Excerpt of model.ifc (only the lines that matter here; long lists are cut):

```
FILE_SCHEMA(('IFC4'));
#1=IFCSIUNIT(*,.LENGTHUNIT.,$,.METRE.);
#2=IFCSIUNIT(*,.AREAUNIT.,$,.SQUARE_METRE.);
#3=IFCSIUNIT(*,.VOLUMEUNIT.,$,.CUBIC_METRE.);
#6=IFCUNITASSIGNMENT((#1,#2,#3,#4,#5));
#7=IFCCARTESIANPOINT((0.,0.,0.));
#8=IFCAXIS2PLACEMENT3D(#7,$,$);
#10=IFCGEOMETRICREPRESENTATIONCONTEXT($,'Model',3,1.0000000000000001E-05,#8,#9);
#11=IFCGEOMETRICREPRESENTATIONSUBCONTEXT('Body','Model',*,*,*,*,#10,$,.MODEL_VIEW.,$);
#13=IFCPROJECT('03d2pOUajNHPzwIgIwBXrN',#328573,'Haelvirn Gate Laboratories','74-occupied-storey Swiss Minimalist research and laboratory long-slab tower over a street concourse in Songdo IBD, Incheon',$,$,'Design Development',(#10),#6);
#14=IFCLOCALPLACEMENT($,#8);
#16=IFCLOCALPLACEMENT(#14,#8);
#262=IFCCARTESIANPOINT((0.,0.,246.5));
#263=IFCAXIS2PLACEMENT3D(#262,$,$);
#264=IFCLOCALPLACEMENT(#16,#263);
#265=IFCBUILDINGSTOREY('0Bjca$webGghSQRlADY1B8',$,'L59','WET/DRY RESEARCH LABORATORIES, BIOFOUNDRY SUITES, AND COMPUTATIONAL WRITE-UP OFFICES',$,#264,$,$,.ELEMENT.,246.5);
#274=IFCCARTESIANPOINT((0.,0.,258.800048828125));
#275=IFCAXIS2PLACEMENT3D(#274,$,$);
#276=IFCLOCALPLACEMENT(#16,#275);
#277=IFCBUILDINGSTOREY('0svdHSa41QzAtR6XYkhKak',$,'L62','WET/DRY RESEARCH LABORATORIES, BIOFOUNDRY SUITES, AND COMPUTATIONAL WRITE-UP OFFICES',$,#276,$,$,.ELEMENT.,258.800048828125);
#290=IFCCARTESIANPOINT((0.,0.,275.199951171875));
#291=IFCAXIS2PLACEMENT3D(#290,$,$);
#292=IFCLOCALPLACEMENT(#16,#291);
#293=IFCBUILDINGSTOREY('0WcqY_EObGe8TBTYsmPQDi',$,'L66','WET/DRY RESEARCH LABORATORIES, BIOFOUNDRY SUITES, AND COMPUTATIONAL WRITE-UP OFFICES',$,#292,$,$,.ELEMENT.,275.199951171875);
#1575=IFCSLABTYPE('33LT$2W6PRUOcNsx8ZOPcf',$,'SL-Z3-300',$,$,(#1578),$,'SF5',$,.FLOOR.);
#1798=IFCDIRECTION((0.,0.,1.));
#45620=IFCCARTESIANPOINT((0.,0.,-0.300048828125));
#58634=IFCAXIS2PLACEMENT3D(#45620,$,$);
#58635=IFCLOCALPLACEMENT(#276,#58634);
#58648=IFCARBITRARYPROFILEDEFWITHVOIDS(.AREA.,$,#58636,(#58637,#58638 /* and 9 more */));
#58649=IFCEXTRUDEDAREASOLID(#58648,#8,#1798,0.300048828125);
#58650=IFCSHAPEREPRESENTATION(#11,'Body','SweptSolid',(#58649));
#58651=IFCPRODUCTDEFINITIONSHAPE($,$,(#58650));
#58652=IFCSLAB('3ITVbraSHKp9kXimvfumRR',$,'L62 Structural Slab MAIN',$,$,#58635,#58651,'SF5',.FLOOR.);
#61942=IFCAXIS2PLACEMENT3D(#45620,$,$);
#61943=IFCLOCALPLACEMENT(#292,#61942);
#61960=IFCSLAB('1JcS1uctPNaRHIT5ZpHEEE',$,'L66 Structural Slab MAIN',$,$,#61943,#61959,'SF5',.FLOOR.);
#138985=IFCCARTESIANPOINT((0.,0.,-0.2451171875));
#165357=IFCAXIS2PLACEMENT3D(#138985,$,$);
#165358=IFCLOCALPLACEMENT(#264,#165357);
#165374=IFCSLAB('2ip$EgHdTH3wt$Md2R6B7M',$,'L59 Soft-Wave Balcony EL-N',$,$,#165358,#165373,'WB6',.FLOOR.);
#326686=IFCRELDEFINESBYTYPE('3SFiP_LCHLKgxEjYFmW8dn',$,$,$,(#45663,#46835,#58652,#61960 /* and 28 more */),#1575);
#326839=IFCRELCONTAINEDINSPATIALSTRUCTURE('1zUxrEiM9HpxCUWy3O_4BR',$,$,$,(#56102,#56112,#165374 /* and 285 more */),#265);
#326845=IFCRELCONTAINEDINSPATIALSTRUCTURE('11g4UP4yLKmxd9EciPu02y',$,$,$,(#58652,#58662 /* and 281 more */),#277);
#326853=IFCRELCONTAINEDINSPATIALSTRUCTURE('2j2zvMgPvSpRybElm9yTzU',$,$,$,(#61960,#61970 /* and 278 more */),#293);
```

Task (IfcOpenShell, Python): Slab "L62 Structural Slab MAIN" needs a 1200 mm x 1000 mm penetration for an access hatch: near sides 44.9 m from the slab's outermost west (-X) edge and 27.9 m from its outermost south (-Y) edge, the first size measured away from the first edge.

```python
import numpy as np
import ifcopenshell
import ifcopenshell.api.feature
import ifcopenshell.api.geometry
import ifcopenshell.api.root
import ifcopenshell.geom
import ifcopenshell.util.placement
import ifcopenshell.util.representation
import ifcopenshell.util.shape
import ifcopenshell.util.unit

model = ifcopenshell.open("model.ifc")
unit_scale = ifcopenshell.util.unit.calculate_unit_scale(model)
settings = ifcopenshell.geom.settings()


def volume(element):
    """Net volume in cubic metres, openings subtracted."""
    shape = ifcopenshell.geom.create_shape(settings, element)
    return ifcopenshell.util.shape.get_volume(shape.geometry)


slab = model.by_id(58652)
before = volume(slab)

# Extent in the slab's own axes, in metres. The edges named are its -X and -Y sides.
slab_shape = ifcopenshell.geom.create_shape(settings, slab)
vertices = ifcopenshell.util.shape.get_vertices(slab_shape.geometry)
x_min, y_min, bottom = vertices.min(axis=0)
top = vertices[:, 2].max()

opening = ifcopenshell.api.root.create_entity(model, ifc_class="IfcOpeningElement", name="Access hatch opening", predefined_type="OPENING")
context = ifcopenshell.util.representation.get_context(model, "Model", "Body", "MODEL_VIEW")
width, depth = 1.2, 1
outline = [(0.0, 0.0), (width, 0.0), (width, depth), (0.0, depth), (0.0, 0.0)]
# Overshoot both faces by 50 mm so the cut is clean.
shape = ifcopenshell.api.geometry.add_slab_representation(
    model, context=context, depth=top - bottom + 0.1, polyline=outline
)
ifcopenshell.api.geometry.assign_representation(model, product=opening, representation=shape)

matrix = ifcopenshell.util.placement.get_local_placement(slab.ObjectPlacement)
matrix[:, 3] = matrix @ np.append(np.array([x_min + 44.9, y_min + 27.9, bottom - 0.05]) / unit_scale, 1.0)
ifcopenshell.api.geometry.edit_object_placement(model, product=opening, matrix=matrix, is_si=False)
ifcopenshell.api.feature.add_feature(model, feature=opening, element=slab)

after = volume(slab)

print(f"slab volume {before:.3f} -> {after:.3f} m3")

model.write("model_v2.ifc")
```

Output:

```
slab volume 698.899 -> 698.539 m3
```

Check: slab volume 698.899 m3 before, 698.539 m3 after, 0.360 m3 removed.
